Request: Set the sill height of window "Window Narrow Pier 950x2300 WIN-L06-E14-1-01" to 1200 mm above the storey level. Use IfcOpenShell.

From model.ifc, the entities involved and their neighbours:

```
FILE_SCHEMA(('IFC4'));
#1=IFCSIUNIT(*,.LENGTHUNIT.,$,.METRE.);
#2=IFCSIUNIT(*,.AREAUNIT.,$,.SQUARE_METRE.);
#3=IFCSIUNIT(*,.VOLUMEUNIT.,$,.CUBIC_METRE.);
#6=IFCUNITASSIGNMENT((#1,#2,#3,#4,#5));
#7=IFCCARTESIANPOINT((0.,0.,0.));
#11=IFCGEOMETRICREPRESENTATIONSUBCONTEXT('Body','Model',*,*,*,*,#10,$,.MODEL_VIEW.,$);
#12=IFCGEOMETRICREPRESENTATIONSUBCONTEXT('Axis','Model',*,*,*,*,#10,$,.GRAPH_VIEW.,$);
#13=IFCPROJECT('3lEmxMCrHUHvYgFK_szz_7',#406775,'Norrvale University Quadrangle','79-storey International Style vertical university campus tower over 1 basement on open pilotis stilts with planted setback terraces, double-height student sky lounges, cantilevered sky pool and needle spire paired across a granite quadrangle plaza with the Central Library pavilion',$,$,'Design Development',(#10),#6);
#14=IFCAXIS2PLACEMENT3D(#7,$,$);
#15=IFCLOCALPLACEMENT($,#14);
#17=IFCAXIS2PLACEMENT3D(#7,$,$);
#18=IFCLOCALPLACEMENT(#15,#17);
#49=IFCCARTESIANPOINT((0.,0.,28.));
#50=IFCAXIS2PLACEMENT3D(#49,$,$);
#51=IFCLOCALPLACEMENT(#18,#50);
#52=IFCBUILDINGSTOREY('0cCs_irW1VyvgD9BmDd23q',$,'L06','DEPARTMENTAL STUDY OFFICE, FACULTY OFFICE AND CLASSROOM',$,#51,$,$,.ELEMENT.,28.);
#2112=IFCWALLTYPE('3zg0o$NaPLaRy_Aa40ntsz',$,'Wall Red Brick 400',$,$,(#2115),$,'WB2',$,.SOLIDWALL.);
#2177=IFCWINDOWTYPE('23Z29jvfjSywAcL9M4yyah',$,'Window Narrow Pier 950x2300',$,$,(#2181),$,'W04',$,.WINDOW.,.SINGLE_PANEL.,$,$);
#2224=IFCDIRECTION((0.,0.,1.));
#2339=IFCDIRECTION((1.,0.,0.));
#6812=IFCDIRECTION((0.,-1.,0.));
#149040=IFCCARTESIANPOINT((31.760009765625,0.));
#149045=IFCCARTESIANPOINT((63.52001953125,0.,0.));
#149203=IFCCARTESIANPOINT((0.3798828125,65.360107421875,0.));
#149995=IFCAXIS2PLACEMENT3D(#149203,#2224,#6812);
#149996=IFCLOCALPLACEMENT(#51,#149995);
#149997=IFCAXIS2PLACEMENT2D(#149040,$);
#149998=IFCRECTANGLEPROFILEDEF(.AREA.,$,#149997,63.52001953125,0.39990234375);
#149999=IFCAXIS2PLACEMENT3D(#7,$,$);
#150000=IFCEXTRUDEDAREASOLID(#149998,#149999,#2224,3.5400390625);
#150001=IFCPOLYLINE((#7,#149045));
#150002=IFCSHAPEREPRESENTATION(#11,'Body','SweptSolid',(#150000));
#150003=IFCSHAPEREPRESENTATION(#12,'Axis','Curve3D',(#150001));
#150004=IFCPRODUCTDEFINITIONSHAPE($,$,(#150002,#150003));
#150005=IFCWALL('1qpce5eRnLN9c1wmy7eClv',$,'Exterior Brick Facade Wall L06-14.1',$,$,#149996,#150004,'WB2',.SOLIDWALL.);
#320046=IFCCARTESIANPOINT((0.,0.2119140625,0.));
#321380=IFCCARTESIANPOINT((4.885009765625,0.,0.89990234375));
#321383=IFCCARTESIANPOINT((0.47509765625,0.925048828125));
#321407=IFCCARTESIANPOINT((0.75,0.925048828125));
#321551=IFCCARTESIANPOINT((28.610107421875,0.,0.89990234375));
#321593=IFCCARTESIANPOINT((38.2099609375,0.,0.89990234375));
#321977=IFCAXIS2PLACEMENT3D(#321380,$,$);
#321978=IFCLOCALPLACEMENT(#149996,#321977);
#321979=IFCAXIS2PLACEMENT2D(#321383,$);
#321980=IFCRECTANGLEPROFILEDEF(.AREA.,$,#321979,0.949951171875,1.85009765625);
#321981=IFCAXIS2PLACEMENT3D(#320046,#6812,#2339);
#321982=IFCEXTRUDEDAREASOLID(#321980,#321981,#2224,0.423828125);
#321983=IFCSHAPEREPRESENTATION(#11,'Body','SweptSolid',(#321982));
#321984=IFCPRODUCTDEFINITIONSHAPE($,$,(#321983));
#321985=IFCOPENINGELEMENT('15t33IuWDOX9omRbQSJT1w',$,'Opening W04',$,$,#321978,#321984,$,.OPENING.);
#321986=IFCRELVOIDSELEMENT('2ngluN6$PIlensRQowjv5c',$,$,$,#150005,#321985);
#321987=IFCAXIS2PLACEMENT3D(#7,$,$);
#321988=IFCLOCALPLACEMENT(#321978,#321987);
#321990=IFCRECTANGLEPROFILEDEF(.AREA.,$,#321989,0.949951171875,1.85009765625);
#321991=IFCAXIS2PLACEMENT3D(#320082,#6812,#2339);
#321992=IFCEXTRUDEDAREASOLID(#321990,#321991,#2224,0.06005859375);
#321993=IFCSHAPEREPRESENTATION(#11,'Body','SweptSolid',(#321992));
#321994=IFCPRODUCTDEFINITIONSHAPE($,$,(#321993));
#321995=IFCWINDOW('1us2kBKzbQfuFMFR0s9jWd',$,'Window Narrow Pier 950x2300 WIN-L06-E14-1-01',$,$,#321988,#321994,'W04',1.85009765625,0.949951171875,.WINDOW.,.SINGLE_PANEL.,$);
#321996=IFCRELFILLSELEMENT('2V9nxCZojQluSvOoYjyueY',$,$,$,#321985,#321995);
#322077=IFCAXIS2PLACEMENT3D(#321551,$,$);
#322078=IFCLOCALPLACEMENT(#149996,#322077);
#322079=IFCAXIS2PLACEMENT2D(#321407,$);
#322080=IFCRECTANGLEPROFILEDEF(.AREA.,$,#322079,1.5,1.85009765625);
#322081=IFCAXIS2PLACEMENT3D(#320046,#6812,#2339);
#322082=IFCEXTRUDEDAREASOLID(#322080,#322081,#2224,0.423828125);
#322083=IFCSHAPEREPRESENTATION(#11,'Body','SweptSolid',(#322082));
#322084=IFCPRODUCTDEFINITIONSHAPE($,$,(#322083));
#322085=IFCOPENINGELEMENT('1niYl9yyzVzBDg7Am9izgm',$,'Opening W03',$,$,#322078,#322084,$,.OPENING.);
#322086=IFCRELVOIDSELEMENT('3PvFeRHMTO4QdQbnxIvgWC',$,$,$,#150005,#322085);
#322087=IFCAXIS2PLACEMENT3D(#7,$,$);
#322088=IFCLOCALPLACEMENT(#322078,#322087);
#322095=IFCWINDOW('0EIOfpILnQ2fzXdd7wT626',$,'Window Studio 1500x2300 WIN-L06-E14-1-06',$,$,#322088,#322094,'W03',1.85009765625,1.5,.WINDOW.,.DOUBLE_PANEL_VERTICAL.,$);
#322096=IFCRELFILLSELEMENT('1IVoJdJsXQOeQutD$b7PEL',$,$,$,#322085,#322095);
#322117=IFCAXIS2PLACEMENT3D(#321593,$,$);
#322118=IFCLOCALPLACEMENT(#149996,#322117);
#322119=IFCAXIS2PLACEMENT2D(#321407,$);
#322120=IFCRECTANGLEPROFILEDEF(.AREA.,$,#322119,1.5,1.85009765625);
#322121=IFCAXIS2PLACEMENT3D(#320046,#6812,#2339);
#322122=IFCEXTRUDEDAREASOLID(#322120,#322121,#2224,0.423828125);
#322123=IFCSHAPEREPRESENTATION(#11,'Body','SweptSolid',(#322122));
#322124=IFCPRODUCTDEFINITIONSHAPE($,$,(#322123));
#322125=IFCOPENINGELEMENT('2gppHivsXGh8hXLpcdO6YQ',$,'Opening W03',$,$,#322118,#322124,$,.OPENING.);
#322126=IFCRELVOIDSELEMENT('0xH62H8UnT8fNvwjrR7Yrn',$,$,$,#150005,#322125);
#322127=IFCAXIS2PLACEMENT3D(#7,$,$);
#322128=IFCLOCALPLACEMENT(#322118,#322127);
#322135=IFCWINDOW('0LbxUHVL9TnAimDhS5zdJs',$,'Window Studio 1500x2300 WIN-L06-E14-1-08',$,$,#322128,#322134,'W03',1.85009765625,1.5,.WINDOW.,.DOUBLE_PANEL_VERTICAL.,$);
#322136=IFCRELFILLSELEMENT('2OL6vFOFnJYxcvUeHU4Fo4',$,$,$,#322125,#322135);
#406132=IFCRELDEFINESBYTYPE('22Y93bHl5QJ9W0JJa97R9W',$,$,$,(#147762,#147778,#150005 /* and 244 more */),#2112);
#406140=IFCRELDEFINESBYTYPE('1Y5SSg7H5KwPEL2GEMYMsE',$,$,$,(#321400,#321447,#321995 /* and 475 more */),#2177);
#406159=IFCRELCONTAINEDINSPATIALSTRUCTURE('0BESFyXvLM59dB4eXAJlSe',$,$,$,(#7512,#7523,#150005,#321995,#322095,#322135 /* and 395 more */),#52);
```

```python
import numpy as np
import ifcopenshell
import ifcopenshell.api.geometry
import ifcopenshell.geom
import ifcopenshell.util.element
import ifcopenshell.util.placement
import ifcopenshell.util.shape
import ifcopenshell.util.unit

model = ifcopenshell.open("model.ifc")
unit_scale = ifcopenshell.util.unit.calculate_unit_scale(model)

window = model.by_guid("1us2kBKzbQfuFMFR0s9jWd")
opening = window.FillsVoids[0].RelatingOpeningElement
storey = ifcopenshell.util.element.get_container(window, ifc_class="IfcBuildingStorey")
level = ifcopenshell.util.placement.get_local_placement(storey.ObjectPlacement)[2, 3]

# The opening's origin need not be at the sill, so measure its lowest point.
shape = ifcopenshell.geom.create_shape(ifcopenshell.geom.settings(), opening)
bottom = ifcopenshell.util.shape.get_shape_bottom_elevation(shape, shape.geometry) / unit_scale
dz = level + 1.2 / unit_scale - bottom

shift = np.array([0.0, 0.0, dz])
# The window is placed relative to its opening, so it follows when the opening moves.
matrix = ifcopenshell.util.placement.get_local_placement(opening.ObjectPlacement)
matrix[:3, 3] += shift
ifcopenshell.api.geometry.edit_object_placement(
    model, product=opening, matrix=matrix, is_si=False, should_transform_children=True
)

print(f"moved by {dz * unit_scale:+.3f} m")

model.write("model_rev.ifc")
```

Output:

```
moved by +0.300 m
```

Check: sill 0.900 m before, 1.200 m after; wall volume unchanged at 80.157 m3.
